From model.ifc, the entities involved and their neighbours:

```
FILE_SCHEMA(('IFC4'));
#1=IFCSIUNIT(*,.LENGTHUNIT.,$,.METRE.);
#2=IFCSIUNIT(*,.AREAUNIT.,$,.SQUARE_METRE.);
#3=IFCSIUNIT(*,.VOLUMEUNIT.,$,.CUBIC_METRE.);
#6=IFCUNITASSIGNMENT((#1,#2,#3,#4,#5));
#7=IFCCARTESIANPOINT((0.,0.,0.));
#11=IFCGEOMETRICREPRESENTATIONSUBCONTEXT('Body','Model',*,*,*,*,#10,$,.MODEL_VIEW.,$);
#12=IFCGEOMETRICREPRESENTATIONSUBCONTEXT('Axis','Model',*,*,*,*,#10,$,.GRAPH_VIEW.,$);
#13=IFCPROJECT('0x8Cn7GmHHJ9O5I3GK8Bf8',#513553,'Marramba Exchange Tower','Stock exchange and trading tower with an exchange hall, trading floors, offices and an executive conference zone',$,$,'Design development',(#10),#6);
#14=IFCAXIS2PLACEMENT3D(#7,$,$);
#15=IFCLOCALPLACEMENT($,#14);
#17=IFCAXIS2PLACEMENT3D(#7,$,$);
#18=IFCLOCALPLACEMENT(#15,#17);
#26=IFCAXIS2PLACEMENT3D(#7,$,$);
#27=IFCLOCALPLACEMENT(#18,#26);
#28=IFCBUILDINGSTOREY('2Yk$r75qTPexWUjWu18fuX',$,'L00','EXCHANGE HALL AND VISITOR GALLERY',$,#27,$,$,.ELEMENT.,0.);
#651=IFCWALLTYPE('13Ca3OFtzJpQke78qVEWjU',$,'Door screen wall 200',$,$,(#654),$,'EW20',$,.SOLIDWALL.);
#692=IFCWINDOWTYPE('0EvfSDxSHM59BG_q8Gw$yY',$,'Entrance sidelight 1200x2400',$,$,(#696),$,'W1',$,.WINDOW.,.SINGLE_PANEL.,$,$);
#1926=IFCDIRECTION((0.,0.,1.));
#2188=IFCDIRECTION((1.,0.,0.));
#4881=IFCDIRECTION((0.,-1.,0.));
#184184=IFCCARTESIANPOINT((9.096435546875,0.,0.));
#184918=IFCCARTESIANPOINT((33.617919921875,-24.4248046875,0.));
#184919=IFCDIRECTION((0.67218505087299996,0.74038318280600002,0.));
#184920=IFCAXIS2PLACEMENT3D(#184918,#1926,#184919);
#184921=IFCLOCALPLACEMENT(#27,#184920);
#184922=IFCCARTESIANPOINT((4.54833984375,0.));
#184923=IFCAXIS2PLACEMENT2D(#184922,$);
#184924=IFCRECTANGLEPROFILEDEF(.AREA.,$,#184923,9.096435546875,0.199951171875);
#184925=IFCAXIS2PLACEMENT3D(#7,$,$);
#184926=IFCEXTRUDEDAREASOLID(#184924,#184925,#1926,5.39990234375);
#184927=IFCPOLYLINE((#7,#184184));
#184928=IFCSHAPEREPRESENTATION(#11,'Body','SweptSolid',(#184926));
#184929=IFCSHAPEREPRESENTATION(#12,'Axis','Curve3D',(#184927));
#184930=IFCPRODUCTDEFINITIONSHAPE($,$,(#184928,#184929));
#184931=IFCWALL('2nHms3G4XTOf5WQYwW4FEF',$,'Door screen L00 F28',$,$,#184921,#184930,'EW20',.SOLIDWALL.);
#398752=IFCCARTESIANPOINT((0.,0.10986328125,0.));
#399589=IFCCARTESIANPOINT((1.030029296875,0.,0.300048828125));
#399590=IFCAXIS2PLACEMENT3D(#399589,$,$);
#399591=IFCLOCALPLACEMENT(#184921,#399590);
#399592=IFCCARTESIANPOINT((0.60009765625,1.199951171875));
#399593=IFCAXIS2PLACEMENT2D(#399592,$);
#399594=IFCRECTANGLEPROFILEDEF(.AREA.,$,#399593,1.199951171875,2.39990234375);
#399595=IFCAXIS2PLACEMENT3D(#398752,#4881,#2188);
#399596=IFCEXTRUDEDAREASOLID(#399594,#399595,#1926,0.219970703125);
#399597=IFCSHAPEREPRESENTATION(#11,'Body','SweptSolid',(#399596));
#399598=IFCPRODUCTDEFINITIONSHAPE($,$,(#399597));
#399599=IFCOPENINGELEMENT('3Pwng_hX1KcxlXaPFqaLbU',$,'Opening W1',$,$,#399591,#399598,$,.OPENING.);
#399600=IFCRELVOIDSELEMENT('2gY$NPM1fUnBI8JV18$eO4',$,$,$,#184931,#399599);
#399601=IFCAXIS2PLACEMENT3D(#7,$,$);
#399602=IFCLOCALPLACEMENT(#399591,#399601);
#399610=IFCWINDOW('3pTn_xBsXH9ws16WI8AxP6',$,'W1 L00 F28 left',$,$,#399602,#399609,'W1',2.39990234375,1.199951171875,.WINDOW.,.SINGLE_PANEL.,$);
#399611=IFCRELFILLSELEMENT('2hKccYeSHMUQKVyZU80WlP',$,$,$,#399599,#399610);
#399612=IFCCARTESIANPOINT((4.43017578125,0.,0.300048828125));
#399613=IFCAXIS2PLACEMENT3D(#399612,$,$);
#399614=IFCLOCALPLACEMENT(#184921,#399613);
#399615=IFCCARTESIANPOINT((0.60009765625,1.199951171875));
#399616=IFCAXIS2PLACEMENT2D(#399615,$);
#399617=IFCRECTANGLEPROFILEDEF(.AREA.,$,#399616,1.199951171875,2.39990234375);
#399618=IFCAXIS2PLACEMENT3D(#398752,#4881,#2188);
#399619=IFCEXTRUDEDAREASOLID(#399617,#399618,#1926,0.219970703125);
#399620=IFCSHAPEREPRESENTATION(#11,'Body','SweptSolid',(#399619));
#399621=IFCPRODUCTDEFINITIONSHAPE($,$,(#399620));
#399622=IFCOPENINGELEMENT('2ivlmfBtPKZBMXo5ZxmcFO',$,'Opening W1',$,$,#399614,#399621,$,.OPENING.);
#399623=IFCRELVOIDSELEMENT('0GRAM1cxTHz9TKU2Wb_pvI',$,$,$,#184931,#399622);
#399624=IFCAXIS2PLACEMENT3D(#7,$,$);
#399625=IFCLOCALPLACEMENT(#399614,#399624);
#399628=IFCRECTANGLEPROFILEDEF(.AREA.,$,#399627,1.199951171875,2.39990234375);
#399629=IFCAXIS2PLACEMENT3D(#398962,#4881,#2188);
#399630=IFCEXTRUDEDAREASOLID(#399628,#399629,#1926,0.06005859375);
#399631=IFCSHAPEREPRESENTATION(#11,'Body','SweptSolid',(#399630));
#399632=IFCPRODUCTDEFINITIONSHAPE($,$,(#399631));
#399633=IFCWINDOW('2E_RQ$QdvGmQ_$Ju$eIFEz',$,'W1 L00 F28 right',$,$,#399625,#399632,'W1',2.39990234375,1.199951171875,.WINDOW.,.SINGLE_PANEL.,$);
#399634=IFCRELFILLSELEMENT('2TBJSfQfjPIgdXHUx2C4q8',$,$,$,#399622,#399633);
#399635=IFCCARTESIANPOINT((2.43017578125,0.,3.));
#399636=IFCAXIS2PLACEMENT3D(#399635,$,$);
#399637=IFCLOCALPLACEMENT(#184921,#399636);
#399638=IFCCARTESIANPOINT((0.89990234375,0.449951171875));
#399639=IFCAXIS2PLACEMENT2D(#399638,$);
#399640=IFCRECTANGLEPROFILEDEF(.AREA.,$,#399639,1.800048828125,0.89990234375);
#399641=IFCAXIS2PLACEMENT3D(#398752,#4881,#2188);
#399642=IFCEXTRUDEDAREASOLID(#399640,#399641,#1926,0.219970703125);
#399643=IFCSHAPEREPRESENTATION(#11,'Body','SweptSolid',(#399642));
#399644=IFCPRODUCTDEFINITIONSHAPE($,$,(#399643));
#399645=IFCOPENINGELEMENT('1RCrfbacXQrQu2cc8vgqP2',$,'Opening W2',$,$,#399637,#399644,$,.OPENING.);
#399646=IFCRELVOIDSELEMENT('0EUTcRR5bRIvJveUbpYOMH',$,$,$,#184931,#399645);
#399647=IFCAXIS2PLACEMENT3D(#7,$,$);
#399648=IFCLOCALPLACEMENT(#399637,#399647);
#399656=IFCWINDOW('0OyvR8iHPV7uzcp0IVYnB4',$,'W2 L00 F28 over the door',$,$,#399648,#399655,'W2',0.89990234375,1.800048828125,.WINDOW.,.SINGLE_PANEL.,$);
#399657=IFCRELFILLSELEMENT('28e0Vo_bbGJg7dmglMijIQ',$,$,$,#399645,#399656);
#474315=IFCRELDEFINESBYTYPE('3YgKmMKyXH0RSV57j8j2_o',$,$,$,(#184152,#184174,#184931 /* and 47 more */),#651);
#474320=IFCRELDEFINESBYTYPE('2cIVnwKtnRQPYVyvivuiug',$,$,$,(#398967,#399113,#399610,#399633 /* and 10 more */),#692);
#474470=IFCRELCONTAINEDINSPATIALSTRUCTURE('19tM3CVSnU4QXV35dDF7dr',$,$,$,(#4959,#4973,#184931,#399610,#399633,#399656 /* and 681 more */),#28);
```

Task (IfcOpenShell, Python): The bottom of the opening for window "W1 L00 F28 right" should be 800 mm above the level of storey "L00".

```python
import numpy as np
import ifcopenshell
import ifcopenshell.api.geometry
import ifcopenshell.geom
import ifcopenshell.util.element
import ifcopenshell.util.placement
import ifcopenshell.util.shape
import ifcopenshell.util.unit

model = ifcopenshell.open("model.ifc")
unit_scale = ifcopenshell.util.unit.calculate_unit_scale(model)

window = model.by_guid("2E_RQ$QdvGmQ_$Ju$eIFEz")
opening = window.FillsVoids[0].RelatingOpeningElement
storey = ifcopenshell.util.element.get_container(window, ifc_class="IfcBuildingStorey")
level = ifcopenshell.util.placement.get_local_placement(storey.ObjectPlacement)[2, 3]

# The opening's origin need not be at the sill, so measure its lowest point.
shape = ifcopenshell.geom.create_shape(ifcopenshell.geom.settings(), opening)
bottom = ifcopenshell.util.shape.get_shape_bottom_elevation(shape, shape.geometry) / unit_scale
dz = level + 0.8 / unit_scale - bottom

shift = np.array([0.0, 0.0, dz])
# The window is placed relative to its opening, so it follows when the opening moves.
matrix = ifcopenshell.util.placement.get_local_placement(opening.ObjectPlacement)
matrix[:3, 3] += shift
ifcopenshell.api.geometry.edit_object_placement(
    model, product=opening, matrix=matrix, is_si=False, should_transform_children=True
)

print(f"moved by {dz * unit_scale:+.3f} m")

model.write("model_v2.ifc")
```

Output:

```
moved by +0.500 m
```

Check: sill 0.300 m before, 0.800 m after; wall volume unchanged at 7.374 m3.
